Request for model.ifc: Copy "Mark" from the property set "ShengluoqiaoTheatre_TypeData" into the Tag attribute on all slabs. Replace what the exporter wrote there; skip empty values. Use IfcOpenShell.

First a look at what the model holds.

```python
import ifcopenshell
import ifcopenshell.util.element

model = ifcopenshell.open("model.ifc")
print(model.schema)
slabs = model.by_type("IfcSlab")
print(len(slabs), "slabs")
for e in slabs[:8]:
    source = ifcopenshell.util.element.get_pset(e, "ShengluoqiaoTheatre_TypeData", "Mark")
    target = e.Tag
    print(e.id(), repr(source), repr(target), sep=" | ")
```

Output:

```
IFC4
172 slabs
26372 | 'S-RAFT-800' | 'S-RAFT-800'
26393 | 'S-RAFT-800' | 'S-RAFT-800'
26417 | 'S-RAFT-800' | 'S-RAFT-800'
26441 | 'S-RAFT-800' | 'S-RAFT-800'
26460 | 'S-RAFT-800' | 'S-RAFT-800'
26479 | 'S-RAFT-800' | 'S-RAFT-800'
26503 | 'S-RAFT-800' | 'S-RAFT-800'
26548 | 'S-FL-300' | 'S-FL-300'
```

```python
import ifcopenshell
import ifcopenshell.util.element

model = ifcopenshell.open("model.ifc")

count = 0
for e in model.by_type("IfcSlab"):
    value = ifcopenshell.util.element.get_pset(e, "ShengluoqiaoTheatre_TypeData", "Mark")
    current = e.Tag
    if not value or not value.strip() or current == value:
        continue
    e.Tag = value
    count += 1

print(count, "slabs updated")

model.write("model_rev.ifc")
```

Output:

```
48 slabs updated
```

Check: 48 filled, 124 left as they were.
